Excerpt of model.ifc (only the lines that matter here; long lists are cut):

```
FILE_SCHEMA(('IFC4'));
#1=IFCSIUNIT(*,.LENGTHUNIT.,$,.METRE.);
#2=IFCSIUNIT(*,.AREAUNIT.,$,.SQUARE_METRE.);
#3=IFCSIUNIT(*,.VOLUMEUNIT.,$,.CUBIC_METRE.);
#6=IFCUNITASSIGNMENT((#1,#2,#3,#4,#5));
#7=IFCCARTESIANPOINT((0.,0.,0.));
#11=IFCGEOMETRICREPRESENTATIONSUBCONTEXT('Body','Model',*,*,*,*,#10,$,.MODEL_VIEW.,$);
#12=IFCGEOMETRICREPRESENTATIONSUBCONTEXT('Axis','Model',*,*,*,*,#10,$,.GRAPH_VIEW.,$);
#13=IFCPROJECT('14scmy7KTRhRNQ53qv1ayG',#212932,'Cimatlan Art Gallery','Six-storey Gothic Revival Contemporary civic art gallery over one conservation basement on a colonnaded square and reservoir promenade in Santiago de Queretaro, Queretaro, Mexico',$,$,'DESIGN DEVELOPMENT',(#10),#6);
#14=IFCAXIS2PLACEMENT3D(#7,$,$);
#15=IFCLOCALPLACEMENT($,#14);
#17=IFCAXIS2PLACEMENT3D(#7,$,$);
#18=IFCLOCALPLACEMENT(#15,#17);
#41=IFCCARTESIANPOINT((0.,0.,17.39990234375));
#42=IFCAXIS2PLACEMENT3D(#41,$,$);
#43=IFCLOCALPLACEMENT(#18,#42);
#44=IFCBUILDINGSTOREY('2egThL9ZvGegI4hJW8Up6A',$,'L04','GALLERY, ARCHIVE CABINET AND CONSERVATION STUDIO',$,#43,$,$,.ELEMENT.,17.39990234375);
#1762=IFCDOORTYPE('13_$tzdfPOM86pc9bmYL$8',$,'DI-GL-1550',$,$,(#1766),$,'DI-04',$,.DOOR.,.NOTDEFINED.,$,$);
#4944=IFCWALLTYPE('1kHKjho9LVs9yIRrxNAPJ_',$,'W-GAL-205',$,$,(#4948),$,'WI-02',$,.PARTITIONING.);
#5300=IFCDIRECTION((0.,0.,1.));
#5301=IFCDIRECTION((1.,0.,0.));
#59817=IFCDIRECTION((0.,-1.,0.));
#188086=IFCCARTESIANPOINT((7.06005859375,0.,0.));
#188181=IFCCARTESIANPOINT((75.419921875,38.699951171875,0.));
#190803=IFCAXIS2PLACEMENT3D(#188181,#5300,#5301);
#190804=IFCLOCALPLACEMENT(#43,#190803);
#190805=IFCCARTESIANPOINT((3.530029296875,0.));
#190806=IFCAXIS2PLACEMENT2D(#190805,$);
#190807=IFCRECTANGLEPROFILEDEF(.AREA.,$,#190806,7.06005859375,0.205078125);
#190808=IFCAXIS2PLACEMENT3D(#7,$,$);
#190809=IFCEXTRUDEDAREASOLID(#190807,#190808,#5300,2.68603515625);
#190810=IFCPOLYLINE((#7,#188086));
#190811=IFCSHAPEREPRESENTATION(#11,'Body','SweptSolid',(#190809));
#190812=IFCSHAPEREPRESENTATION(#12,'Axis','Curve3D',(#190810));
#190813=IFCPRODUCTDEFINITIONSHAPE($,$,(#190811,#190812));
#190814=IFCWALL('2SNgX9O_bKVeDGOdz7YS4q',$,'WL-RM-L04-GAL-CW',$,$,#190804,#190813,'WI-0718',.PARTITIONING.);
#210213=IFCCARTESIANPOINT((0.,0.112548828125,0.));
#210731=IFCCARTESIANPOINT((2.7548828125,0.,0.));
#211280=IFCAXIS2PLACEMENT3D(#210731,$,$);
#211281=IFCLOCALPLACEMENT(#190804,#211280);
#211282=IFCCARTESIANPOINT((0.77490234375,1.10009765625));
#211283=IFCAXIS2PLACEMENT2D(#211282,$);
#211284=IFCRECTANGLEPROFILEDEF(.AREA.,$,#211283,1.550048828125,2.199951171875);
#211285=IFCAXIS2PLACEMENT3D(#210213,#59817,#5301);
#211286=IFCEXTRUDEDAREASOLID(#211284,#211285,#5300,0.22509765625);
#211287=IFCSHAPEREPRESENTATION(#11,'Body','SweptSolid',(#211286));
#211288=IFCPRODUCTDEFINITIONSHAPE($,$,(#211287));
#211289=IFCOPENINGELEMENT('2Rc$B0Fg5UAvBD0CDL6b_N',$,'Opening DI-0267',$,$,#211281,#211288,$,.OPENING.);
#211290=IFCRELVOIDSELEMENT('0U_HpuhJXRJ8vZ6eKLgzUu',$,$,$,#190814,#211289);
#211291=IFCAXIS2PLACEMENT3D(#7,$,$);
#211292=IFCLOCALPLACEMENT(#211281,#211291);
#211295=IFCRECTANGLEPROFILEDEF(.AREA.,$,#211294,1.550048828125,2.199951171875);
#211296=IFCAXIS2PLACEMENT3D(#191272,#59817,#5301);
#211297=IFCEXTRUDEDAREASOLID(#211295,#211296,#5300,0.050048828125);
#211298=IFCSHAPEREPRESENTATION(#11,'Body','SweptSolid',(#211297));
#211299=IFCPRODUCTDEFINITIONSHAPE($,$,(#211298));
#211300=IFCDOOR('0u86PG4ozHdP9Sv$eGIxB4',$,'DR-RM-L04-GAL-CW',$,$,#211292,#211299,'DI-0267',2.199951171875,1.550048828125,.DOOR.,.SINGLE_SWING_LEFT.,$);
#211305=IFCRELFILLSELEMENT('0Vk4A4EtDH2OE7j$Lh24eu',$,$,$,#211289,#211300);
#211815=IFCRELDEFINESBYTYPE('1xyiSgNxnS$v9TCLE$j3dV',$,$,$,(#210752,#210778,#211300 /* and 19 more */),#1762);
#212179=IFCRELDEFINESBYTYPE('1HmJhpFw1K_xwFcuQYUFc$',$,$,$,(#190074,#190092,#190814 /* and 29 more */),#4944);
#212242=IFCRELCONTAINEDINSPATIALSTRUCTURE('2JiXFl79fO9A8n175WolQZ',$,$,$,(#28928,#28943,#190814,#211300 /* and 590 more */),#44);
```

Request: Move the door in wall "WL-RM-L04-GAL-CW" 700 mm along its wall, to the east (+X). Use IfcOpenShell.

```python
import ifcopenshell
import ifcopenshell.api.geometry
import ifcopenshell.util.placement
import ifcopenshell.util.unit

model = ifcopenshell.open("model.ifc")
unit_scale = ifcopenshell.util.unit.calculate_unit_scale(model)

door = model.by_guid("0u86PG4ozHdP9Sv$eGIxB4")
opening = door.FillsVoids[0].RelatingOpeningElement
wall = opening.VoidsElements[0].RelatingBuildingElement

wall_matrix = ifcopenshell.util.placement.get_local_placement(wall.ObjectPlacement)
shift = wall_matrix[:3, 0] * 0.7 / unit_scale
before = ifcopenshell.util.placement.get_local_placement(door.ObjectPlacement)[:3, 3].copy()

# The door is placed relative to its opening, so it follows when the opening moves.
matrix = ifcopenshell.util.placement.get_local_placement(opening.ObjectPlacement)
matrix[:3, 3] += shift
ifcopenshell.api.geometry.edit_object_placement(
    model, product=opening, matrix=matrix, is_si=False, should_transform_children=True
)

after = ifcopenshell.util.placement.get_local_placement(door.ObjectPlacement)[:3, 3]
print("door moved by", (after - before).round(3) + 0.0)

model.write("model-out.ifc")
```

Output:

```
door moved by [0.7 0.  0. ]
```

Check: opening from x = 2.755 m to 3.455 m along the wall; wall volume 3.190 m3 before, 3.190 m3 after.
